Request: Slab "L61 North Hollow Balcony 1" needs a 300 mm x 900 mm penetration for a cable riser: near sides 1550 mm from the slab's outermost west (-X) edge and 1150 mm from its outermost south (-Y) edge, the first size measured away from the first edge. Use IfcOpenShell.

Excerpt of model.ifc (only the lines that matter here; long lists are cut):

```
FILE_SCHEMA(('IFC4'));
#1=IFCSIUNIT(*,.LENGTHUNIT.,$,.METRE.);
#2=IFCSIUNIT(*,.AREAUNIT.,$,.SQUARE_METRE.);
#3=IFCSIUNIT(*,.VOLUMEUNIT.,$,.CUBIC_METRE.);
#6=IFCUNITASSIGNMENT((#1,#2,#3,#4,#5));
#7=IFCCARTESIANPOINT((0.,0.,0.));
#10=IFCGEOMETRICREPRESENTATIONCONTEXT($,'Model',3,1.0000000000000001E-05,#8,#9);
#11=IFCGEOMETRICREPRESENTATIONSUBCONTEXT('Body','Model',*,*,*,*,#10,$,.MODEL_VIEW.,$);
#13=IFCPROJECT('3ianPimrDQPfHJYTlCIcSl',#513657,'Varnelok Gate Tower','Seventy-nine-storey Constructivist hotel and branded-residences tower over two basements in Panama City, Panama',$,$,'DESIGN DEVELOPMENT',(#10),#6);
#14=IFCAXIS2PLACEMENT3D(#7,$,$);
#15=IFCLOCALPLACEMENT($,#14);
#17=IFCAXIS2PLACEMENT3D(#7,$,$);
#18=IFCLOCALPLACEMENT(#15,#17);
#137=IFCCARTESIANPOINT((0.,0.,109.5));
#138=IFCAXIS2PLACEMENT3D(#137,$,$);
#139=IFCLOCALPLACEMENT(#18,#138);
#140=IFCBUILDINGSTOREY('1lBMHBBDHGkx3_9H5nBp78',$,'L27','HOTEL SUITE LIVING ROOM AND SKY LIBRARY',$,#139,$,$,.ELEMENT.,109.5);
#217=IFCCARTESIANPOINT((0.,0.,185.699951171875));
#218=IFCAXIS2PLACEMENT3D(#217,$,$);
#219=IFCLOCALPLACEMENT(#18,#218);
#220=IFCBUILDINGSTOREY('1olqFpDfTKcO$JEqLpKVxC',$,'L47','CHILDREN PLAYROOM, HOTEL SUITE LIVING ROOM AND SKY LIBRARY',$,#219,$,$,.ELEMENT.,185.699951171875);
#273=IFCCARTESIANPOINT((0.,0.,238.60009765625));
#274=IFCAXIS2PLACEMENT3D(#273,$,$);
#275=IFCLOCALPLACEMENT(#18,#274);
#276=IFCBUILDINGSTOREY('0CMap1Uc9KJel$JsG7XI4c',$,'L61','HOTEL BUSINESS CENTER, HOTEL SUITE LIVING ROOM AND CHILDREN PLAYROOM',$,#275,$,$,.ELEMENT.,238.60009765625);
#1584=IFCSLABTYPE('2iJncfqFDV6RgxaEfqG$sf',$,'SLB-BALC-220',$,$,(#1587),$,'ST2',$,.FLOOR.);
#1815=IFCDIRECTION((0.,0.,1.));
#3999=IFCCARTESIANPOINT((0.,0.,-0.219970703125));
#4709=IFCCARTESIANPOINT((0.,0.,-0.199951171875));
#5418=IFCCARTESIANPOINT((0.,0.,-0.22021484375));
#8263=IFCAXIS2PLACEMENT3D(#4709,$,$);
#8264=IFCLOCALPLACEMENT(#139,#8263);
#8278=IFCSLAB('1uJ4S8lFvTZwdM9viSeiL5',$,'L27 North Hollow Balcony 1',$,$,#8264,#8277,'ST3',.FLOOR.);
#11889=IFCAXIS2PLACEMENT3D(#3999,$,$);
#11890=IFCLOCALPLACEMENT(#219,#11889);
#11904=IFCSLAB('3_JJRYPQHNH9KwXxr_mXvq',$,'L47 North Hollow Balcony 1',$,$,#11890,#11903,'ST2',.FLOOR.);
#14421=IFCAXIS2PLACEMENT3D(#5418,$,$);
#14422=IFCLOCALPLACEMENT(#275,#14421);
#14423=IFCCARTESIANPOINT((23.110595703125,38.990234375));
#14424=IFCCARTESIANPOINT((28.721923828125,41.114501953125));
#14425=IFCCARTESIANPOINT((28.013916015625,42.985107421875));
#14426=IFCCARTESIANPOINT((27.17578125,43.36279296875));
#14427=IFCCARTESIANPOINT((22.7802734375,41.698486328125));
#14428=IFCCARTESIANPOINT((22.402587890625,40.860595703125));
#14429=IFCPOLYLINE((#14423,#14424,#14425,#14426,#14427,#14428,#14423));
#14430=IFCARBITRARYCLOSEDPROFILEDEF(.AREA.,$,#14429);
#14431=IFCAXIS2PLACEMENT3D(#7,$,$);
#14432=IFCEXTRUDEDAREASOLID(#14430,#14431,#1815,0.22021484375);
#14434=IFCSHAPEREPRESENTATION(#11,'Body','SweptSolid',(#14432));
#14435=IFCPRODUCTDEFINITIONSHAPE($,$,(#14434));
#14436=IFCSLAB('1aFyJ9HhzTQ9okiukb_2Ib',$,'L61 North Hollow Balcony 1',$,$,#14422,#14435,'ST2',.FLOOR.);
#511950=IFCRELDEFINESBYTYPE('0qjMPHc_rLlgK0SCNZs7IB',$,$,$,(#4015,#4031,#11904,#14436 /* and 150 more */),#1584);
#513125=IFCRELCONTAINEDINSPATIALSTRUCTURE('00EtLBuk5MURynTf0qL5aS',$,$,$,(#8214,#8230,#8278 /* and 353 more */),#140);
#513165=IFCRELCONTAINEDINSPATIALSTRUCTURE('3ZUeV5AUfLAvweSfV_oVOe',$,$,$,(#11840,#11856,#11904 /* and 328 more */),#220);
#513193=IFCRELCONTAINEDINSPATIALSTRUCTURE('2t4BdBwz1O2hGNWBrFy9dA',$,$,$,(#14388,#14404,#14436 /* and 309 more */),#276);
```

```python
import numpy as np
import ifcopenshell
import ifcopenshell.api.feature
import ifcopenshell.api.geometry
import ifcopenshell.api.root
import ifcopenshell.geom
import ifcopenshell.util.placement
import ifcopenshell.util.representation
import ifcopenshell.util.shape
import ifcopenshell.util.unit

model = ifcopenshell.open("model.ifc")
unit_scale = ifcopenshell.util.unit.calculate_unit_scale(model)
settings = ifcopenshell.geom.settings()


def volume(element):
    """Net volume in cubic metres, openings subtracted."""
    shape = ifcopenshell.geom.create_shape(settings, element)
    return ifcopenshell.util.shape.get_volume(shape.geometry)


slab = model.by_guid("1aFyJ9HhzTQ9okiukb_2Ib")
before = volume(slab)

# Extent in the slab's own axes, in metres. The edges named are its -X and -Y sides.
slab_shape = ifcopenshell.geom.create_shape(settings, slab)
vertices = ifcopenshell.util.shape.get_vertices(slab_shape.geometry)
x_min, y_min, bottom = vertices.min(axis=0)
top = vertices[:, 2].max()

opening = ifcopenshell.api.root.create_entity(model, ifc_class="IfcOpeningElement", name="Cable riser opening", predefined_type="OPENING")
context = ifcopenshell.util.representation.get_context(model, "Model", "Body", "MODEL_VIEW")
width, depth = 0.3, 0.9
outline = [(0.0, 0.0), (width, 0.0), (width, depth), (0.0, depth), (0.0, 0.0)]
# Overshoot both faces by 50 mm so the cut is clean.
shape = ifcopenshell.api.geometry.add_slab_representation(
    model, context=context, depth=top - bottom + 0.1, polyline=outline
)
ifcopenshell.api.geometry.assign_representation(model, product=opening, representation=shape)

matrix = ifcopenshell.util.placement.get_local_placement(slab.ObjectPlacement)
matrix[:, 3] = matrix @ np.append(np.array([x_min + 1.55, y_min + 1.15, bottom - 0.05]) / unit_scale, 1.0)
ifcopenshell.api.geometry.edit_object_placement(model, product=opening, matrix=matrix, is_si=False)
ifcopenshell.api.feature.add_feature(model, feature=opening, element=slab)

after = volume(slab)

print(f"slab volume {before:.3f} -> {after:.3f} m3")

model.write("model_updated.ifc")
```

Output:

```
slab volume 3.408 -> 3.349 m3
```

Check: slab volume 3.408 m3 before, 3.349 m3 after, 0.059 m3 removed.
